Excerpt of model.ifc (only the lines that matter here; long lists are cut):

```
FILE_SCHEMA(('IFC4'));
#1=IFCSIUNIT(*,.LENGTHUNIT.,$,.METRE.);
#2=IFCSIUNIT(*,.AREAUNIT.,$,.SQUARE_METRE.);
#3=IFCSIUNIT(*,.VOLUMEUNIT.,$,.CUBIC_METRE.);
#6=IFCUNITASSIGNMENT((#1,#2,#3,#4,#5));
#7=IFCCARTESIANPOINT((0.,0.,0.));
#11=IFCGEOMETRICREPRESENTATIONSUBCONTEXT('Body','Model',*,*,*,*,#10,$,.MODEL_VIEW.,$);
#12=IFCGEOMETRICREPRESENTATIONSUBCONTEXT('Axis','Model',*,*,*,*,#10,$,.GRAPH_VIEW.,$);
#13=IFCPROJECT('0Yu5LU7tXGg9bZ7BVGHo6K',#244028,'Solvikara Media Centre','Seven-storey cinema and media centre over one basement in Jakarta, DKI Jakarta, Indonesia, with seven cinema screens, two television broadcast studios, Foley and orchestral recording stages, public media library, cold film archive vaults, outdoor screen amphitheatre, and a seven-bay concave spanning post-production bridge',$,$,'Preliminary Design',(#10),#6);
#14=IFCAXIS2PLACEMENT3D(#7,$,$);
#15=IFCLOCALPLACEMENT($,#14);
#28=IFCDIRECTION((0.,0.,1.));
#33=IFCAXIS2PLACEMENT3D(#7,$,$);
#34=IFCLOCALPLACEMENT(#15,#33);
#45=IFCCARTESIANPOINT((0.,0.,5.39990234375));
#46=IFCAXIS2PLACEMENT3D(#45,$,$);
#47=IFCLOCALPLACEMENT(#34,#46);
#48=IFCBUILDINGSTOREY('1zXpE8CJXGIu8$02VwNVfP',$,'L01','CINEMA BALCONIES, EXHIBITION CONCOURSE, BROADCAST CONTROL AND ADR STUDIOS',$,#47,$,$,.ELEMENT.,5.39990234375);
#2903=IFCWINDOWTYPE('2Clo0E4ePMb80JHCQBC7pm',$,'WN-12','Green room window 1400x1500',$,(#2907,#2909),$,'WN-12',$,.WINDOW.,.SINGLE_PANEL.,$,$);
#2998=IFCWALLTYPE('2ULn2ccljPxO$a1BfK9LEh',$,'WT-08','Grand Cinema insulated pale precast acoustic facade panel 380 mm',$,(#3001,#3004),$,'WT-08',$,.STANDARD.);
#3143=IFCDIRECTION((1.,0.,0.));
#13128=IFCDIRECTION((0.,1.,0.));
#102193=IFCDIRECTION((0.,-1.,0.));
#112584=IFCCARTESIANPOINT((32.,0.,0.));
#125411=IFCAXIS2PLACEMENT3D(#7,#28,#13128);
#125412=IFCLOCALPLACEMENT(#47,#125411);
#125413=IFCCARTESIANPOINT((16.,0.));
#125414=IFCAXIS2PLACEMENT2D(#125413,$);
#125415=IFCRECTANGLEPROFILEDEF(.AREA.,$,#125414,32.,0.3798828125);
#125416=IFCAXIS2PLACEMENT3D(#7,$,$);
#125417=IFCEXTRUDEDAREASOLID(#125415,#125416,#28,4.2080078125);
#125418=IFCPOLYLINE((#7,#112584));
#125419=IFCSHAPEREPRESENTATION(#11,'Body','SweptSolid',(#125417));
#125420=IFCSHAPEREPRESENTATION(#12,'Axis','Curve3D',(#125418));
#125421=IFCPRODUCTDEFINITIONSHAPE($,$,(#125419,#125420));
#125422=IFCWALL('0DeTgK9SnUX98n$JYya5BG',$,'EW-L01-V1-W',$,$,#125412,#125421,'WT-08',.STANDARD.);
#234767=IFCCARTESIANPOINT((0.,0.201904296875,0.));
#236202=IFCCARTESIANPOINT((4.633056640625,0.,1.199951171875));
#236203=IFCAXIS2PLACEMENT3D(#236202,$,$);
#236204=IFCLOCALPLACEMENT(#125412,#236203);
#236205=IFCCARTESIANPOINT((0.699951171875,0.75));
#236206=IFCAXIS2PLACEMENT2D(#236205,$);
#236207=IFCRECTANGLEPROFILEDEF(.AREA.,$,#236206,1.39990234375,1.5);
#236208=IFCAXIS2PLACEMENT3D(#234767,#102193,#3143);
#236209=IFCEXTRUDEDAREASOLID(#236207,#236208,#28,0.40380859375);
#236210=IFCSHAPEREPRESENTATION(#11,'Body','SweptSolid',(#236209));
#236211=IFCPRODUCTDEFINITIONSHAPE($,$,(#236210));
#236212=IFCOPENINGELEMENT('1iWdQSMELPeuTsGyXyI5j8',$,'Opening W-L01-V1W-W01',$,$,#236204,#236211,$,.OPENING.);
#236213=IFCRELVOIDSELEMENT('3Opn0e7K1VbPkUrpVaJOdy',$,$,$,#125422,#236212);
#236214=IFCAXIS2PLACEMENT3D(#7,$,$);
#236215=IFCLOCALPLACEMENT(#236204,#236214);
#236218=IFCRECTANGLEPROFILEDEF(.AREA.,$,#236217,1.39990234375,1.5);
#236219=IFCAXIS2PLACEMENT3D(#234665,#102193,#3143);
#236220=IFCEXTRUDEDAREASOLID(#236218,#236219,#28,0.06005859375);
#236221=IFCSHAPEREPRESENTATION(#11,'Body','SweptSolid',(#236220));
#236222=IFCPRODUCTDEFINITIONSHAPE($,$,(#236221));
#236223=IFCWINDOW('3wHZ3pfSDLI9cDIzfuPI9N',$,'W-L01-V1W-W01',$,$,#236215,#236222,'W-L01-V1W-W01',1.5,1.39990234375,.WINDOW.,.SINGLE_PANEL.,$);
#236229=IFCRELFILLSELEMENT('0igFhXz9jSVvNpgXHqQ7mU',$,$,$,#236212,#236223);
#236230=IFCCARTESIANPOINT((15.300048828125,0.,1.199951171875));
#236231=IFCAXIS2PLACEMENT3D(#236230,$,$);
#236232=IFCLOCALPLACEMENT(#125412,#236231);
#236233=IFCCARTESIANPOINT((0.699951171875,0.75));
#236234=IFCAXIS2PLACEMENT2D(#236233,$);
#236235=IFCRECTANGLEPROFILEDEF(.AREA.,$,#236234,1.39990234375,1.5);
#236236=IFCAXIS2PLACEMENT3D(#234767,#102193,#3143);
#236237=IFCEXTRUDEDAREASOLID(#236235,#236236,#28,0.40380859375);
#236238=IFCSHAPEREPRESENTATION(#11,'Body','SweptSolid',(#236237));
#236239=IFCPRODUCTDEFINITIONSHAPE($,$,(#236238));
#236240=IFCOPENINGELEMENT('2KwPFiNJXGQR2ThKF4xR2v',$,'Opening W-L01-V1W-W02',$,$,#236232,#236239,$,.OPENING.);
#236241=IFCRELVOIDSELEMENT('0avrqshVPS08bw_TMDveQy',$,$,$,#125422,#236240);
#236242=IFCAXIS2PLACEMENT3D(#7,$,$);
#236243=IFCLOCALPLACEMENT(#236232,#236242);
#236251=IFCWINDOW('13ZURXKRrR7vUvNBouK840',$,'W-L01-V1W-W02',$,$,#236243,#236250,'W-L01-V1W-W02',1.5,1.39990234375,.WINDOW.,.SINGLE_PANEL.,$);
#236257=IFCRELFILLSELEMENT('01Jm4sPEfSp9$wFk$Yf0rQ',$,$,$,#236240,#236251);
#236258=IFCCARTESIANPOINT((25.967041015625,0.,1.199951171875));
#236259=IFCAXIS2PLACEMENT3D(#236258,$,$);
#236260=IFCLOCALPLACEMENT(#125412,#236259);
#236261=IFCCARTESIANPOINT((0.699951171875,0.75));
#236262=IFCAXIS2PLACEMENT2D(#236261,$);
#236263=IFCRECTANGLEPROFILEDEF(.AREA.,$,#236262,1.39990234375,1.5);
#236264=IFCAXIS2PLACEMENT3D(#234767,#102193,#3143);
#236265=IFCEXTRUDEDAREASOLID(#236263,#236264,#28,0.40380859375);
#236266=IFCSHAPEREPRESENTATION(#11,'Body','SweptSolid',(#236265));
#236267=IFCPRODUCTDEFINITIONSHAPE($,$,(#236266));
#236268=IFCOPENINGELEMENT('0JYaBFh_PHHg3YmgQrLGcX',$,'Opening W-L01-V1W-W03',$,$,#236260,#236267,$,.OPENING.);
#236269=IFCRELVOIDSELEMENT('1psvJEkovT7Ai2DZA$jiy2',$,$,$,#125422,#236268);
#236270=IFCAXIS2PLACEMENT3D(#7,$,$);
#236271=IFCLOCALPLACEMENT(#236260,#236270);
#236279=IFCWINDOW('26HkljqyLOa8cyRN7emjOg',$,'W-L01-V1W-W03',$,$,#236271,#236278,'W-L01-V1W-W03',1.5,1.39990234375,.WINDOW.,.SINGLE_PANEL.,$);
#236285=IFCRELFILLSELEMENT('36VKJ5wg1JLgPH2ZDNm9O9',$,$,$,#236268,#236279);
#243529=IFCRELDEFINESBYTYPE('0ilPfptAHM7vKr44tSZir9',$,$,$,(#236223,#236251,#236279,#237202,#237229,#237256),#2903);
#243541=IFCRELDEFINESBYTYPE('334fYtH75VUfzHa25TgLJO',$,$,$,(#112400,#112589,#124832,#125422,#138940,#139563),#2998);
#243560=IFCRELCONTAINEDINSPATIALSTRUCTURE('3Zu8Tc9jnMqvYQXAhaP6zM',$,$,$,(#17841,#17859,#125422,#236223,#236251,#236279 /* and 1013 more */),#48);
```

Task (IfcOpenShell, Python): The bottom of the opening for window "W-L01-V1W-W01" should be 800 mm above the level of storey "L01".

```python
import numpy as np
import ifcopenshell
import ifcopenshell.api.geometry
import ifcopenshell.geom
import ifcopenshell.util.element
import ifcopenshell.util.placement
import ifcopenshell.util.shape
import ifcopenshell.util.unit

model = ifcopenshell.open("model.ifc")
unit_scale = ifcopenshell.util.unit.calculate_unit_scale(model)

window = model.by_guid("3wHZ3pfSDLI9cDIzfuPI9N")
opening = window.FillsVoids[0].RelatingOpeningElement
storey = ifcopenshell.util.element.get_container(window, ifc_class="IfcBuildingStorey")
level = ifcopenshell.util.placement.get_local_placement(storey.ObjectPlacement)[2, 3]

# The opening's origin need not be at the sill, so measure its lowest point.
shape = ifcopenshell.geom.create_shape(ifcopenshell.geom.settings(), opening)
bottom = ifcopenshell.util.shape.get_shape_bottom_elevation(shape, shape.geometry) / unit_scale
dz = level + 0.8 - bottom

shift = np.array([0.0, 0.0, dz])
# The window is placed relative to its opening, so it follows when the opening moves.
matrix = ifcopenshell.util.placement.get_local_placement(opening.ObjectPlacement)
matrix[:3, 3] += shift
ifcopenshell.api.geometry.edit_object_placement(
    model, product=opening, matrix=matrix, is_si=False, should_transform_children=True
)

print(f"moved by {dz * unit_scale:+.3f} m")

model.write("model_v2.ifc")
```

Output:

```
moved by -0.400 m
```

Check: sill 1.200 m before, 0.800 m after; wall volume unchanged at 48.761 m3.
